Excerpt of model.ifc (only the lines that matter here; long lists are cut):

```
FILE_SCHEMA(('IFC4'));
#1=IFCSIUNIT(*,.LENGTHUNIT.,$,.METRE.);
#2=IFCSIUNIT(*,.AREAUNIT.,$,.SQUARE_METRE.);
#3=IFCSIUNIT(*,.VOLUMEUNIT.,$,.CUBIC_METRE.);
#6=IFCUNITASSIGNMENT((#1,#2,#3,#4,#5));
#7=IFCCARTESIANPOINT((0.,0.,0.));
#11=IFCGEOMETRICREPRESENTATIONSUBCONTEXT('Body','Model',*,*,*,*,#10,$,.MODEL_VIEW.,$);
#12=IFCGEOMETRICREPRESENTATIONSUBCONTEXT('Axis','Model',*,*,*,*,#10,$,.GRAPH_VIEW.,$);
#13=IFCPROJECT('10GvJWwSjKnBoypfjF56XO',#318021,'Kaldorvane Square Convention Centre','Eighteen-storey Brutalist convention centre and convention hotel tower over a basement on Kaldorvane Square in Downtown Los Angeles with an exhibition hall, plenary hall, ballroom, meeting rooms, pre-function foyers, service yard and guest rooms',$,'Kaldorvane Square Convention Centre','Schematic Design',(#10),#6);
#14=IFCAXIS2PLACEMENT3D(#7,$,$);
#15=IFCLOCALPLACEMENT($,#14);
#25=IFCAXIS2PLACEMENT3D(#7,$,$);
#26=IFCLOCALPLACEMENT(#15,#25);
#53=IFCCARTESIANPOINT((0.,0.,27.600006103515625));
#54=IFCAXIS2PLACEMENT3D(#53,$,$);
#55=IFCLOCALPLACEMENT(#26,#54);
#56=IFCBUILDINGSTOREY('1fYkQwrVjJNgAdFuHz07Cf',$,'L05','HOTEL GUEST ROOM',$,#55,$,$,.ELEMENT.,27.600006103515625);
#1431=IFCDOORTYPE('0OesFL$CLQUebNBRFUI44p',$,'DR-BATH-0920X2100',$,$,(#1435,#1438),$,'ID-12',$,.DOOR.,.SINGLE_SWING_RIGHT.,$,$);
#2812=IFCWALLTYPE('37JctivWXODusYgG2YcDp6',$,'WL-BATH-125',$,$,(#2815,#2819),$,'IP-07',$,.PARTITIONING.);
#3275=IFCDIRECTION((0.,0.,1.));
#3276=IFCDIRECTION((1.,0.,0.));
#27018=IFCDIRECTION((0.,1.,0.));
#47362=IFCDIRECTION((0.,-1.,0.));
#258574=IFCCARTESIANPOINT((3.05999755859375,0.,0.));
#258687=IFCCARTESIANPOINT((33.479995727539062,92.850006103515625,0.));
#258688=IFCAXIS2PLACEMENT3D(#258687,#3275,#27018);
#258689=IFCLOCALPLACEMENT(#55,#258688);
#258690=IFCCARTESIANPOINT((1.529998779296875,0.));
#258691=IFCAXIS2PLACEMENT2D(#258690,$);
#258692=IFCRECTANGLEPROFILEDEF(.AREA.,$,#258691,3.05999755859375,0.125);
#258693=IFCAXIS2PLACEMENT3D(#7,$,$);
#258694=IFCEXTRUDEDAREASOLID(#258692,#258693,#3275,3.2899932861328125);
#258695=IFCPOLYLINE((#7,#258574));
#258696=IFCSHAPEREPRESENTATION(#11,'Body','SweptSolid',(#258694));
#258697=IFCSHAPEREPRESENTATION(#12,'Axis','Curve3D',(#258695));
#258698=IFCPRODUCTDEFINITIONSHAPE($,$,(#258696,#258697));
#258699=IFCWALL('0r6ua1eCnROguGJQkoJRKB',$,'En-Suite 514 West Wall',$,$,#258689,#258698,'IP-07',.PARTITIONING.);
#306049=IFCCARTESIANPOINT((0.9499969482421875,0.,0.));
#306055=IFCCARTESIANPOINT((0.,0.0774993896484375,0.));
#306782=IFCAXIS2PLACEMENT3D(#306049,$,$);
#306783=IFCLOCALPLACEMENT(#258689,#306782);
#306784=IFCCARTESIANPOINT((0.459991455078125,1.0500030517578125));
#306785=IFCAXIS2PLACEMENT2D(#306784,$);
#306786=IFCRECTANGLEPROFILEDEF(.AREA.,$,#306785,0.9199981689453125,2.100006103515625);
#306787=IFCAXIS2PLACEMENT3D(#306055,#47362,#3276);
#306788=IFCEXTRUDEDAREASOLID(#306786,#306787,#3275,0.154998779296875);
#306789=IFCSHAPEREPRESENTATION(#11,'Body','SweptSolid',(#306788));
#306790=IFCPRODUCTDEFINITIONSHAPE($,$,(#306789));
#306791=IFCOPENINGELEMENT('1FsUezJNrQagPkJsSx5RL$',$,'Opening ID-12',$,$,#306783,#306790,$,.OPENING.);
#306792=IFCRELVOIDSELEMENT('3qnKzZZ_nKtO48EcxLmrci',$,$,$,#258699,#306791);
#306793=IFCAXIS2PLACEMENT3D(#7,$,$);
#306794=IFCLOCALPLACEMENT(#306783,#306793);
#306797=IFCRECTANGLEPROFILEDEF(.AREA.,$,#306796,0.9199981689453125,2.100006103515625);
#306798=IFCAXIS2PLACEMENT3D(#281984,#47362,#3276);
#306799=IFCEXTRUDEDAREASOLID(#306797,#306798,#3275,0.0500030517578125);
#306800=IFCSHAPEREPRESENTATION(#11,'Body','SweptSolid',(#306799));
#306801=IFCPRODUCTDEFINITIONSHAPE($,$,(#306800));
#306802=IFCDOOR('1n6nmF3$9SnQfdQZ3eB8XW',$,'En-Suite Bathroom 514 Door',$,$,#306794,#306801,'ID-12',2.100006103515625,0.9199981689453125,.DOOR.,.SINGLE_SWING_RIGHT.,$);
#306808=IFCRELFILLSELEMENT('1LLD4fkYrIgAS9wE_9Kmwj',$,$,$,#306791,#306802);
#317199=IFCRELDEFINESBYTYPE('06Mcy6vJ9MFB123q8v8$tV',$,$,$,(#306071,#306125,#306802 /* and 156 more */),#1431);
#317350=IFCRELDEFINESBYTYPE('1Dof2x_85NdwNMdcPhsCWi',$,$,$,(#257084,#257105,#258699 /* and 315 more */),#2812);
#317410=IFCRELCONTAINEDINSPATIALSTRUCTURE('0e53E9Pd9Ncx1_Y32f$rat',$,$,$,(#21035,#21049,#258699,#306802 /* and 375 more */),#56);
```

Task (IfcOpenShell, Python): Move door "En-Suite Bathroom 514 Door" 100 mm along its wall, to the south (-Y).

```python
import ifcopenshell
import ifcopenshell.api.geometry
import ifcopenshell.util.placement
import ifcopenshell.util.unit

model = ifcopenshell.open("model.ifc")
unit_scale = ifcopenshell.util.unit.calculate_unit_scale(model)

door = model.by_id(306802)
opening = door.FillsVoids[0].RelatingOpeningElement
wall = opening.VoidsElements[0].RelatingBuildingElement

wall_matrix = ifcopenshell.util.placement.get_local_placement(wall.ObjectPlacement)
shift = wall_matrix[:3, 0] * -0.1 / unit_scale
before = ifcopenshell.util.placement.get_local_placement(door.ObjectPlacement)[:3, 3].copy()

# The door is placed relative to its opening, so it follows when the opening moves.
matrix = ifcopenshell.util.placement.get_local_placement(opening.ObjectPlacement)
matrix[:3, 3] += shift
ifcopenshell.api.geometry.edit_object_placement(
    model, product=opening, matrix=matrix, is_si=False, should_transform_children=True
)

after = ifcopenshell.util.placement.get_local_placement(door.ObjectPlacement)[:3, 3]
print("door moved by", (after - before).round(3) + 0.0)

model.write("model_v2.ifc")
```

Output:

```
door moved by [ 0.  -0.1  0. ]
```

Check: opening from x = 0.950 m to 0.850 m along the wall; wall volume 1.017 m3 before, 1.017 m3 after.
